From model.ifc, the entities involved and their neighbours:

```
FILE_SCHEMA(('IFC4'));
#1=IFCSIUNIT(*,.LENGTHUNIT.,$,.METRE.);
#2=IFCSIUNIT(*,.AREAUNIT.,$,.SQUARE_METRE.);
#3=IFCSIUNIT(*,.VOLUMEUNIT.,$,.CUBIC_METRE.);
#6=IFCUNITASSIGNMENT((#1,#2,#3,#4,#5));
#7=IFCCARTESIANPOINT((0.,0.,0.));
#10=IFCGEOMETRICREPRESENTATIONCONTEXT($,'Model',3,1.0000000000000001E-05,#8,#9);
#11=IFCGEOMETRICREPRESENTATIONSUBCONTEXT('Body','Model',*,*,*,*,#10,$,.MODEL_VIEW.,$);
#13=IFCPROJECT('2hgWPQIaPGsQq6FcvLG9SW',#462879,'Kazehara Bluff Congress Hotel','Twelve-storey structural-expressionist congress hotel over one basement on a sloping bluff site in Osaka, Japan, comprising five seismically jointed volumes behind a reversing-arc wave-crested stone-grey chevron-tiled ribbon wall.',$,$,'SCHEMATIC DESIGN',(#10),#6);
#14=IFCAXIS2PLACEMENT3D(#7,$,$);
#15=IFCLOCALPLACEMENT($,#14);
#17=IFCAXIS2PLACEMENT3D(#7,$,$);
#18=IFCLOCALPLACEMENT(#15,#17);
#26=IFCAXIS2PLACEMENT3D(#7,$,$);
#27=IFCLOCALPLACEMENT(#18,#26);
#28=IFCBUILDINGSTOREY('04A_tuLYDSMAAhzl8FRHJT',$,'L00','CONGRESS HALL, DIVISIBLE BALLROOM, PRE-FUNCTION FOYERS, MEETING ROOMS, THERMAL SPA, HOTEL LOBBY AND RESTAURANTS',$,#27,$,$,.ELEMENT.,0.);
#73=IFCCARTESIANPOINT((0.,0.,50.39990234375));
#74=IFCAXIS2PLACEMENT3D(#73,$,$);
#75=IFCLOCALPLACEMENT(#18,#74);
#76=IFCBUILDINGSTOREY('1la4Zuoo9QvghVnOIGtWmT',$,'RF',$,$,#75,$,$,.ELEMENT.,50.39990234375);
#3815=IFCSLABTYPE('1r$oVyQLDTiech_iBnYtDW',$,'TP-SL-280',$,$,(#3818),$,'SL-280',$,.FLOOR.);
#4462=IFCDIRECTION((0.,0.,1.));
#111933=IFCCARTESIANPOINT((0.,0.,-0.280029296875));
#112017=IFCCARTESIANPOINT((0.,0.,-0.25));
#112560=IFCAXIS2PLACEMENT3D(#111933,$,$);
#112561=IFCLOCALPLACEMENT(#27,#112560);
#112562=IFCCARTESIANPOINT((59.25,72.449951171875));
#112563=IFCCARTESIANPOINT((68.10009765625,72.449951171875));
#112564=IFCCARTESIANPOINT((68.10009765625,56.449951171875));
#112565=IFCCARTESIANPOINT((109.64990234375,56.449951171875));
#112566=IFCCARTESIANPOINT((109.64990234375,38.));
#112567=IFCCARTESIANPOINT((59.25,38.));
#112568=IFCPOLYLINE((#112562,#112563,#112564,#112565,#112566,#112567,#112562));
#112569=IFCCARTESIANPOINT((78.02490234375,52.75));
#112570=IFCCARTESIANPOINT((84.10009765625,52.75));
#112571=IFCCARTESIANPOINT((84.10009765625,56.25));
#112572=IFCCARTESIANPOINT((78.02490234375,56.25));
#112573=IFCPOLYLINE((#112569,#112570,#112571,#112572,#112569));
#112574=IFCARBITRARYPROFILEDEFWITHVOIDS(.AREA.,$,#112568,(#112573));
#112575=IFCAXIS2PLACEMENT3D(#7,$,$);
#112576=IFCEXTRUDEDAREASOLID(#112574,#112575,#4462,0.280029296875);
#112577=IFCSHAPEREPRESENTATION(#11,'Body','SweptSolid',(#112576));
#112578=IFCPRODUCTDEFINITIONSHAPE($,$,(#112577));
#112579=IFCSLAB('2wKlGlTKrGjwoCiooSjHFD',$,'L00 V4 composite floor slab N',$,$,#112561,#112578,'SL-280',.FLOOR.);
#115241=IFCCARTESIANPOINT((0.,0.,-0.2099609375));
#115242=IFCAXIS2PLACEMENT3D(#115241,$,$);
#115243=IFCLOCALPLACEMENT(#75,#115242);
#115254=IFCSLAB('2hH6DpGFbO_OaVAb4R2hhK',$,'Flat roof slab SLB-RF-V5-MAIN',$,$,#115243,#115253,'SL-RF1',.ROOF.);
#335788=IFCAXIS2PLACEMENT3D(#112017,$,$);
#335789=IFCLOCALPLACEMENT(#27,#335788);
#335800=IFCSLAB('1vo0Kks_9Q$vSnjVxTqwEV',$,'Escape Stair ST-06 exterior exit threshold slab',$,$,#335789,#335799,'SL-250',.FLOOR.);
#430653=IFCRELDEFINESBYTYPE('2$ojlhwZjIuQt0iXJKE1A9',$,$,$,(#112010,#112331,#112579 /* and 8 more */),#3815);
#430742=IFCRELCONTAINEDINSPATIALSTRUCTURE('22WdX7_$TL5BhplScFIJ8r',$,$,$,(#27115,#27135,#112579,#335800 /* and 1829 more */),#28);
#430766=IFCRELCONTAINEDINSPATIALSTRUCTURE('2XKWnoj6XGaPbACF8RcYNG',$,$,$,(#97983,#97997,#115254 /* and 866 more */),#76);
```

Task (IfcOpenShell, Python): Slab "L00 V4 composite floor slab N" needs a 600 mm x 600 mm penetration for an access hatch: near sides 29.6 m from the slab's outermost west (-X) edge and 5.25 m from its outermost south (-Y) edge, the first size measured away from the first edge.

```python
import numpy as np
import ifcopenshell
import ifcopenshell.api.feature
import ifcopenshell.api.geometry
import ifcopenshell.api.root
import ifcopenshell.geom
import ifcopenshell.util.placement
import ifcopenshell.util.representation
import ifcopenshell.util.shape
import ifcopenshell.util.unit

model = ifcopenshell.open("model.ifc")
unit_scale = ifcopenshell.util.unit.calculate_unit_scale(model)
settings = ifcopenshell.geom.settings()


def volume(element):
    """Net volume in cubic metres, openings subtracted."""
    shape = ifcopenshell.geom.create_shape(settings, element)
    return ifcopenshell.util.shape.get_volume(shape.geometry)


slab = model.by_guid("2wKlGlTKrGjwoCiooSjHFD")
before = volume(slab)

# Extent in the slab's own axes, in metres. The edges named are its -X and -Y sides.
slab_shape = ifcopenshell.geom.create_shape(settings, slab)
vertices = ifcopenshell.util.shape.get_vertices(slab_shape.geometry)
x_min, y_min, bottom = vertices.min(axis=0)
top = vertices[:, 2].max()

opening = ifcopenshell.api.root.create_entity(model, ifc_class="IfcOpeningElement", name="Access hatch opening", predefined_type="OPENING")
context = ifcopenshell.util.representation.get_context(model, "Model", "Body", "MODEL_VIEW")
width, depth = 0.6, 0.6
outline = [(0.0, 0.0), (width, 0.0), (width, depth), (0.0, depth), (0.0, 0.0)]
# Overshoot both faces by 50 mm so the cut is clean.
shape = ifcopenshell.api.geometry.add_slab_representation(
    model, context=context, depth=top - bottom + 0.1, polyline=outline
)
ifcopenshell.api.geometry.assign_representation(model, product=opening, representation=shape)

matrix = ifcopenshell.util.placement.get_local_placement(slab.ObjectPlacement)
matrix[:, 3] = matrix @ np.append(np.array([x_min + 29.6, y_min + 5.25, bottom - 0.05]) / unit_scale, 1.0)
ifcopenshell.api.geometry.edit_object_placement(model, product=opening, matrix=matrix, is_si=False)
ifcopenshell.api.feature.add_feature(model, feature=opening, element=slab)

after = volume(slab)

print(f"slab volume {before:.3f} -> {after:.3f} m3")

model.write("model_v2.ifc")
```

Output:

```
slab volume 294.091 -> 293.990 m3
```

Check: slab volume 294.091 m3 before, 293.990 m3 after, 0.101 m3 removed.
